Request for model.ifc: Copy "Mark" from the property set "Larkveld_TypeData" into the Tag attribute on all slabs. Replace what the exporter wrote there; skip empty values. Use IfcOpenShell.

First a look at what the model holds.

```python
import ifcopenshell
import ifcopenshell.util.element

model = ifcopenshell.open("model.ifc")
print(model.schema)
slabs = model.by_type("IfcSlab")
print(len(slabs), "slabs")
for e in slabs[:8]:
    source = ifcopenshell.util.element.get_pset(e, "Larkveld_TypeData", "Mark")
    target = e.Tag
    print(e.id(), repr(source), repr(target), sep=" | ")
```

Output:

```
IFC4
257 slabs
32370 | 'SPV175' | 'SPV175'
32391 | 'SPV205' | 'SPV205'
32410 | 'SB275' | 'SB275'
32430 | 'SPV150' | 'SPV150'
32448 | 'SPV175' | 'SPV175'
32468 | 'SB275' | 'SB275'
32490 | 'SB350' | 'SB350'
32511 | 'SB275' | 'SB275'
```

```python
import ifcopenshell
import ifcopenshell.util.element

model = ifcopenshell.open("model.ifc")

count = 0
for e in model.by_type("IfcSlab"):
    value = ifcopenshell.util.element.get_pset(e, "Larkveld_TypeData", "Mark")
    current = e.Tag
    if not value or not value.strip() or current == value:
        continue
    e.Tag = value
    count += 1

print(count, "slabs updated")

model.write("model_updated.ifc")
```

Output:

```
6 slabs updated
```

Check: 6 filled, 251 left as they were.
